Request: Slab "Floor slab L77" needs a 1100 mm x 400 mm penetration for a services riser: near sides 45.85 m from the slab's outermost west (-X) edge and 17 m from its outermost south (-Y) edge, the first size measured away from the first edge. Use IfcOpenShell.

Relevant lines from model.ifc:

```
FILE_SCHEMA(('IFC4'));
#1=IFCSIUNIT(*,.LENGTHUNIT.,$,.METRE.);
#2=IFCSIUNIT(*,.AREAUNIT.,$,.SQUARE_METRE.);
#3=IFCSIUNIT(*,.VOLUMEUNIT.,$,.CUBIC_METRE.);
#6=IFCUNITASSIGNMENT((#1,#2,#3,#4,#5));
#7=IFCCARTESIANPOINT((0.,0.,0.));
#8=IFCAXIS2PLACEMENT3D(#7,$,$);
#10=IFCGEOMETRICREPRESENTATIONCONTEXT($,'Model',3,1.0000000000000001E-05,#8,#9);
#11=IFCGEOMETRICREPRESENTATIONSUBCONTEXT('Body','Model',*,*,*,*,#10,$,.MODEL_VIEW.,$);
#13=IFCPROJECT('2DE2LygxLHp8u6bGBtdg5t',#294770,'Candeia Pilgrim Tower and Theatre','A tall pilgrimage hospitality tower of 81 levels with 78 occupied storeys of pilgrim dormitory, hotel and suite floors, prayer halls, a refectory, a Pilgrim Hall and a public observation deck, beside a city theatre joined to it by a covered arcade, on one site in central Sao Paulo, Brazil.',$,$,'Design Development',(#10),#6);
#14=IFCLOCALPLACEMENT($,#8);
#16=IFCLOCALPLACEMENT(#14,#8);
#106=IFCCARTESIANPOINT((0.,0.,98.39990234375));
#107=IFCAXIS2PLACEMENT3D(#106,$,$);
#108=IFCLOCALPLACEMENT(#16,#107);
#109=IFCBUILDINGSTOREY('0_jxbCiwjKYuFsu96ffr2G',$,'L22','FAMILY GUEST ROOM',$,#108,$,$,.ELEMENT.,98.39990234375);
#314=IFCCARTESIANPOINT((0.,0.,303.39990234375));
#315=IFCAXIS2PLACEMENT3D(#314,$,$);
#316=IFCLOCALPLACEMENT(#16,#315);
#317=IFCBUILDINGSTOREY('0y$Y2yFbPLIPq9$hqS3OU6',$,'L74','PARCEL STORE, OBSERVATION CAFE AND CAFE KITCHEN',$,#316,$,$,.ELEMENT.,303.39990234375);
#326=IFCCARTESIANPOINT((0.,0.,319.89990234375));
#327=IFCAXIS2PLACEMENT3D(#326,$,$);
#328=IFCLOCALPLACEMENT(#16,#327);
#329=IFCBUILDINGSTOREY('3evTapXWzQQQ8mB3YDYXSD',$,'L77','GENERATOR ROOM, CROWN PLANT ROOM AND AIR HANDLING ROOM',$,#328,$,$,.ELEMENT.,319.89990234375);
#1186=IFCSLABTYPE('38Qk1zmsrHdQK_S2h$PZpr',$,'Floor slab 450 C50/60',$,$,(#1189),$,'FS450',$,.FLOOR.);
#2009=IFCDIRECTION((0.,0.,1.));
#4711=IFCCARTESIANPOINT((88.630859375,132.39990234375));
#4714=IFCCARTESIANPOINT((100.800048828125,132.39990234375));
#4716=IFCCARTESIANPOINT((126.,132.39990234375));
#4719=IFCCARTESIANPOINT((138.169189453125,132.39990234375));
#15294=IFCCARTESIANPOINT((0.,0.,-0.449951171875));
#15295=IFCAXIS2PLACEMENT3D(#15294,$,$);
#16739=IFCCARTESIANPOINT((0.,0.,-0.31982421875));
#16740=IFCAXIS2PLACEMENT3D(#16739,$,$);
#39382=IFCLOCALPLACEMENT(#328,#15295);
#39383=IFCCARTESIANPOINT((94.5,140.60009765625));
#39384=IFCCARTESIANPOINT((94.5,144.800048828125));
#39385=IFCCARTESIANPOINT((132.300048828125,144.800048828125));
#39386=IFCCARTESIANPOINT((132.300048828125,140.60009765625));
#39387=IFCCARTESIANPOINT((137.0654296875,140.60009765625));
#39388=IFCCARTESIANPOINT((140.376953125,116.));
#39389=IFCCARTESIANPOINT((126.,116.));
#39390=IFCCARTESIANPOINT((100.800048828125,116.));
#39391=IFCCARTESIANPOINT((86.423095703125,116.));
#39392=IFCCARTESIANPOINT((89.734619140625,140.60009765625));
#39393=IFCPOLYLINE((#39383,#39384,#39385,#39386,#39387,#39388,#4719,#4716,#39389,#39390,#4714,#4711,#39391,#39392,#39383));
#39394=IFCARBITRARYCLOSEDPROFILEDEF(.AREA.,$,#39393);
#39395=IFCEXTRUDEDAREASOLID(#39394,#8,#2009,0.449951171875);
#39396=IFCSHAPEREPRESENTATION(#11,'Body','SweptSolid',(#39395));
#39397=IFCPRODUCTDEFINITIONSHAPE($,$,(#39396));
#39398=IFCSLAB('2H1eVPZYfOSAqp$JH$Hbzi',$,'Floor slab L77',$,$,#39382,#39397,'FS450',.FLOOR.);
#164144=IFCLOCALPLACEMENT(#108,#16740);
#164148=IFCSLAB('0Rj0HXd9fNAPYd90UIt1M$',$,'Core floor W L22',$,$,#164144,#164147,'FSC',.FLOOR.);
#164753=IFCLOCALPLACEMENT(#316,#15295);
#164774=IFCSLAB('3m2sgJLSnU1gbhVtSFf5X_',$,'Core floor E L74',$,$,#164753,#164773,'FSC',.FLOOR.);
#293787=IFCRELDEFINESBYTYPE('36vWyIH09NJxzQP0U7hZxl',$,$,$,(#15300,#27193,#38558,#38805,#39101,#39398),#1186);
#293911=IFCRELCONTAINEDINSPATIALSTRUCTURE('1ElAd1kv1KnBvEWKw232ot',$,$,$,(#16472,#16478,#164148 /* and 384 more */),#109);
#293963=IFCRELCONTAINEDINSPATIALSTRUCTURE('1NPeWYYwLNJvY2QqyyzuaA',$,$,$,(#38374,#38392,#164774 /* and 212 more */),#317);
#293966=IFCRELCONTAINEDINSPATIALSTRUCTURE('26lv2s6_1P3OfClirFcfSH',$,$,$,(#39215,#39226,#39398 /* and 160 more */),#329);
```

```python
import numpy as np
import ifcopenshell
import ifcopenshell.api.feature
import ifcopenshell.api.geometry
import ifcopenshell.api.root
import ifcopenshell.geom
import ifcopenshell.util.placement
import ifcopenshell.util.representation
import ifcopenshell.util.shape
import ifcopenshell.util.unit

model = ifcopenshell.open("model.ifc")
unit_scale = ifcopenshell.util.unit.calculate_unit_scale(model)
settings = ifcopenshell.geom.settings()


def volume(element):
    """Net volume in cubic metres, openings subtracted."""
    shape = ifcopenshell.geom.create_shape(settings, element)
    return ifcopenshell.util.shape.get_volume(shape.geometry)


slab = model.by_guid("2H1eVPZYfOSAqp$JH$Hbzi")
before = volume(slab)

# Extent in the slab's own axes, in metres. The edges named are its -X and -Y sides.
slab_shape = ifcopenshell.geom.create_shape(settings, slab)
vertices = ifcopenshell.util.shape.get_vertices(slab_shape.geometry)
x_min, y_min, bottom = vertices.min(axis=0)
top = vertices[:, 2].max()

opening = ifcopenshell.api.root.create_entity(model, ifc_class="IfcOpeningElement", name="Services riser opening", predefined_type="OPENING")
context = ifcopenshell.util.representation.get_context(model, "Model", "Body", "MODEL_VIEW")
width, depth = 1.1, 0.4
outline = [(0.0, 0.0), (width, 0.0), (width, depth), (0.0, depth), (0.0, 0.0)]
# Overshoot both faces by 50 mm so the cut is clean.
shape = ifcopenshell.api.geometry.add_slab_representation(
    model, context=context, depth=top - bottom + 0.1, polyline=outline
)
ifcopenshell.api.geometry.assign_representation(model, product=opening, representation=shape)

matrix = ifcopenshell.util.placement.get_local_placement(slab.ObjectPlacement)
matrix[:, 3] = matrix @ np.append(np.array([x_min + 45.85, y_min + 17, bottom - 0.05]) / unit_scale, 1.0)
ifcopenshell.api.geometry.edit_object_placement(model, product=opening, matrix=matrix, is_si=False)
ifcopenshell.api.feature.add_feature(model, feature=opening, element=slab)

after = volume(slab)

print(f"slab volume {before:.3f} -> {after:.3f} m3")

model.write("model_updated.ifc")
```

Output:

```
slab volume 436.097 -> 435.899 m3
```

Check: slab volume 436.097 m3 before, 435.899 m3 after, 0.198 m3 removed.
